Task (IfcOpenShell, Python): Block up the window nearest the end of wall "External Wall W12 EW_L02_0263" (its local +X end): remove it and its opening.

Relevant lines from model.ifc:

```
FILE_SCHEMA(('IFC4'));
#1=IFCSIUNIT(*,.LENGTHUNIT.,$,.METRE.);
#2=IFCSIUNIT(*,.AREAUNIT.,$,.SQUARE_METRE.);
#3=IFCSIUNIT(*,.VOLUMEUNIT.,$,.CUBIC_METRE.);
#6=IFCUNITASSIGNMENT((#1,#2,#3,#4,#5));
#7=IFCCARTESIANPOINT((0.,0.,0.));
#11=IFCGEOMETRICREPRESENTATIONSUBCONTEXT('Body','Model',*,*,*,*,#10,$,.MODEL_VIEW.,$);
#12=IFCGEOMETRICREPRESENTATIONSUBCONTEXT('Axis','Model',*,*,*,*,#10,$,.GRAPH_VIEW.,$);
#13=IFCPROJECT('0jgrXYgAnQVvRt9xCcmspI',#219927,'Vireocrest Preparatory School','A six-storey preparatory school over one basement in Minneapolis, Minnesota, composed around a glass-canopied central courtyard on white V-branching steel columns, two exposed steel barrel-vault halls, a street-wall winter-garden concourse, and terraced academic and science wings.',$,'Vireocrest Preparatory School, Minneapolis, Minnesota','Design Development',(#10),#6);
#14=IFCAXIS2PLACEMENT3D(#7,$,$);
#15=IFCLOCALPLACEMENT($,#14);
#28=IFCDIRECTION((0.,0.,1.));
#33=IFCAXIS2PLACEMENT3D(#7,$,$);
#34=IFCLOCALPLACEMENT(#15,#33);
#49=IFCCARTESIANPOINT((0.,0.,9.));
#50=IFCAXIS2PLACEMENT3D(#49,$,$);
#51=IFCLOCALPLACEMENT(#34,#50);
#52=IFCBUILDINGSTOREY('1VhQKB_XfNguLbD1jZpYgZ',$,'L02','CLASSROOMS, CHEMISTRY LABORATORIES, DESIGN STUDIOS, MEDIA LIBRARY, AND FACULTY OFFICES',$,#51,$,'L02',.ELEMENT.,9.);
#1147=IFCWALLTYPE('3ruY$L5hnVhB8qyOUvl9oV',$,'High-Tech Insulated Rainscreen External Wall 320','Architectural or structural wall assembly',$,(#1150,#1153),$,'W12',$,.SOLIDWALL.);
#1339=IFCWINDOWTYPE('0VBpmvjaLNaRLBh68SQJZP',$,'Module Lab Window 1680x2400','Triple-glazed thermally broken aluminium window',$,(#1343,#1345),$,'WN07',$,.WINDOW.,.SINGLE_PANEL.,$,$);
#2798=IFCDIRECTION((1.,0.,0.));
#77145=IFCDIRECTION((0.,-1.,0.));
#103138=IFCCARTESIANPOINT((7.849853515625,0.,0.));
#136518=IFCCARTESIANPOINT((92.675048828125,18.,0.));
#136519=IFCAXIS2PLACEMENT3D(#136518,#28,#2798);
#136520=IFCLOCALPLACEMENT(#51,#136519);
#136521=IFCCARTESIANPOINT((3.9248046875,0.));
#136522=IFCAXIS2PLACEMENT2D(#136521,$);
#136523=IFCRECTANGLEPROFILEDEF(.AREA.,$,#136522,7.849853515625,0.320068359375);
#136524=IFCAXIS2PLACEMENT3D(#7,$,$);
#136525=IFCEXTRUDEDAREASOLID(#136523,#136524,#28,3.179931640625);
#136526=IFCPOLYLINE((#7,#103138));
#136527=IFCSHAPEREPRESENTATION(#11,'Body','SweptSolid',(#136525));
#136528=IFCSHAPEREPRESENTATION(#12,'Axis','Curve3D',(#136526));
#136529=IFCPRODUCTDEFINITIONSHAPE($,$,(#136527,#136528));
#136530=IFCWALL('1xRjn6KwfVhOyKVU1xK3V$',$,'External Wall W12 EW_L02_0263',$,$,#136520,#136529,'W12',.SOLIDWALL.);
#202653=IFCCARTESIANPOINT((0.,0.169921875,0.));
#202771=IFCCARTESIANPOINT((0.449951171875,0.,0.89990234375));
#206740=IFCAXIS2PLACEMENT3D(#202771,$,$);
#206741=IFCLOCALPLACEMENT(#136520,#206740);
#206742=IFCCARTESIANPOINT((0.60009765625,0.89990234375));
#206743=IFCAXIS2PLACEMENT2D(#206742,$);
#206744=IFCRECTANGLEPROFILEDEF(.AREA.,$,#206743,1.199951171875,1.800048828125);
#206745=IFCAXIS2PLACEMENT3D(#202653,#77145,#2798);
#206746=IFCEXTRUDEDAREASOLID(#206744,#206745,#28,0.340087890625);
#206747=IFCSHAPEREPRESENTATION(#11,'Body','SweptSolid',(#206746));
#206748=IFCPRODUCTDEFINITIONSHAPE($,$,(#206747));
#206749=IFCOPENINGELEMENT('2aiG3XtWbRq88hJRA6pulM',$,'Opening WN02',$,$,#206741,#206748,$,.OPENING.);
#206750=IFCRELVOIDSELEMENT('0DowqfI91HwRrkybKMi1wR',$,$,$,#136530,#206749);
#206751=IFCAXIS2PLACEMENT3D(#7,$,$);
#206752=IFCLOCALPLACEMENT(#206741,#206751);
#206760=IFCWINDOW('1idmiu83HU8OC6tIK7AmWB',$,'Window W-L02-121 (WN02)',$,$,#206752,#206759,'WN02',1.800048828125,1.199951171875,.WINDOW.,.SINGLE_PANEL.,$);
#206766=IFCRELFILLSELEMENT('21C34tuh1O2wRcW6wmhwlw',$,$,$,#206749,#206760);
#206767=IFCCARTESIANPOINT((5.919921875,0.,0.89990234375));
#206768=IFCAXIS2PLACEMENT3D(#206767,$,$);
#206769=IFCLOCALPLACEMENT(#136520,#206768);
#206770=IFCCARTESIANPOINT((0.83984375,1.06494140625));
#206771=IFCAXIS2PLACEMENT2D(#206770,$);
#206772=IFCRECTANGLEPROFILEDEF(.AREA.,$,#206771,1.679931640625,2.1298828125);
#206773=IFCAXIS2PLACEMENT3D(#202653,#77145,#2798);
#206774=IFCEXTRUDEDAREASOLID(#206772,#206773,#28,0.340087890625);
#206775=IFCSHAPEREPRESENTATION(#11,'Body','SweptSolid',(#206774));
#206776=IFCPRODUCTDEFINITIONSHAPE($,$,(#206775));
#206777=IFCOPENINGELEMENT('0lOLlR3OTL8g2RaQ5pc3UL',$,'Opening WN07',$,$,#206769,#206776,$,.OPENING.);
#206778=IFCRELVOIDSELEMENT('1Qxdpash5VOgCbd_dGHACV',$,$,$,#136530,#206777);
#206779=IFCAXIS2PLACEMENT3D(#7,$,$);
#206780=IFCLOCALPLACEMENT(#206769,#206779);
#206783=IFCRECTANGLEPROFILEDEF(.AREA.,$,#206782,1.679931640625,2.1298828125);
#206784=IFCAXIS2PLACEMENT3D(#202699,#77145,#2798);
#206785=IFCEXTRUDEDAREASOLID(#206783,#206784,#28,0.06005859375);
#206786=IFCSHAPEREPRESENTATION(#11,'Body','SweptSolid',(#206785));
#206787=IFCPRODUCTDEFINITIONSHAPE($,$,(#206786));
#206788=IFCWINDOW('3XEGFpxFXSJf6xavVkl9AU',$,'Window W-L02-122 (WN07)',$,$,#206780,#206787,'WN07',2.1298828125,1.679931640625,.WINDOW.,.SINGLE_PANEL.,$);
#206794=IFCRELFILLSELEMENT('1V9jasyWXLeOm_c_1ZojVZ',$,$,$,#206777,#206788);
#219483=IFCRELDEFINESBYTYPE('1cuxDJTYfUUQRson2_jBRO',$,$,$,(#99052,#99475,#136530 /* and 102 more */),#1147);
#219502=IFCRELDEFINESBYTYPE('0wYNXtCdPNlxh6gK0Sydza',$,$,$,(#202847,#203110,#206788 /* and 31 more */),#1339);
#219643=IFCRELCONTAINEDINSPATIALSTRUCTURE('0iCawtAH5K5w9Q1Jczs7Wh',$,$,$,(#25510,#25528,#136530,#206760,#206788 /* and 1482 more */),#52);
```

```python
import ifcopenshell
import ifcopenshell.api.feature
import ifcopenshell.api.root
import ifcopenshell.geom
import ifcopenshell.util.shape

model = ifcopenshell.open("model.ifc")
settings = ifcopenshell.geom.settings()


def volume(element):
    """Net volume in cubic metres, openings subtracted."""
    shape = ifcopenshell.geom.create_shape(settings, element)
    return ifcopenshell.util.shape.get_volume(shape.geometry)


window = model.by_guid("3XEGFpxFXSJf6xavVkl9AU")
opening = window.FillsVoids[0].RelatingOpeningElement
wall = opening.VoidsElements[0].RelatingBuildingElement
before = volume(wall)

ifcopenshell.api.root.remove_product(model, product=window)
ifcopenshell.api.feature.remove_feature(model, feature=opening)

after = volume(wall)

print(f"wall volume {before:.3f} -> {after:.3f} m3")

model.write("model-out.ifc")
```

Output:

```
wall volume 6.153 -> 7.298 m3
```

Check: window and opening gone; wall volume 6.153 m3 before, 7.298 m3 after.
